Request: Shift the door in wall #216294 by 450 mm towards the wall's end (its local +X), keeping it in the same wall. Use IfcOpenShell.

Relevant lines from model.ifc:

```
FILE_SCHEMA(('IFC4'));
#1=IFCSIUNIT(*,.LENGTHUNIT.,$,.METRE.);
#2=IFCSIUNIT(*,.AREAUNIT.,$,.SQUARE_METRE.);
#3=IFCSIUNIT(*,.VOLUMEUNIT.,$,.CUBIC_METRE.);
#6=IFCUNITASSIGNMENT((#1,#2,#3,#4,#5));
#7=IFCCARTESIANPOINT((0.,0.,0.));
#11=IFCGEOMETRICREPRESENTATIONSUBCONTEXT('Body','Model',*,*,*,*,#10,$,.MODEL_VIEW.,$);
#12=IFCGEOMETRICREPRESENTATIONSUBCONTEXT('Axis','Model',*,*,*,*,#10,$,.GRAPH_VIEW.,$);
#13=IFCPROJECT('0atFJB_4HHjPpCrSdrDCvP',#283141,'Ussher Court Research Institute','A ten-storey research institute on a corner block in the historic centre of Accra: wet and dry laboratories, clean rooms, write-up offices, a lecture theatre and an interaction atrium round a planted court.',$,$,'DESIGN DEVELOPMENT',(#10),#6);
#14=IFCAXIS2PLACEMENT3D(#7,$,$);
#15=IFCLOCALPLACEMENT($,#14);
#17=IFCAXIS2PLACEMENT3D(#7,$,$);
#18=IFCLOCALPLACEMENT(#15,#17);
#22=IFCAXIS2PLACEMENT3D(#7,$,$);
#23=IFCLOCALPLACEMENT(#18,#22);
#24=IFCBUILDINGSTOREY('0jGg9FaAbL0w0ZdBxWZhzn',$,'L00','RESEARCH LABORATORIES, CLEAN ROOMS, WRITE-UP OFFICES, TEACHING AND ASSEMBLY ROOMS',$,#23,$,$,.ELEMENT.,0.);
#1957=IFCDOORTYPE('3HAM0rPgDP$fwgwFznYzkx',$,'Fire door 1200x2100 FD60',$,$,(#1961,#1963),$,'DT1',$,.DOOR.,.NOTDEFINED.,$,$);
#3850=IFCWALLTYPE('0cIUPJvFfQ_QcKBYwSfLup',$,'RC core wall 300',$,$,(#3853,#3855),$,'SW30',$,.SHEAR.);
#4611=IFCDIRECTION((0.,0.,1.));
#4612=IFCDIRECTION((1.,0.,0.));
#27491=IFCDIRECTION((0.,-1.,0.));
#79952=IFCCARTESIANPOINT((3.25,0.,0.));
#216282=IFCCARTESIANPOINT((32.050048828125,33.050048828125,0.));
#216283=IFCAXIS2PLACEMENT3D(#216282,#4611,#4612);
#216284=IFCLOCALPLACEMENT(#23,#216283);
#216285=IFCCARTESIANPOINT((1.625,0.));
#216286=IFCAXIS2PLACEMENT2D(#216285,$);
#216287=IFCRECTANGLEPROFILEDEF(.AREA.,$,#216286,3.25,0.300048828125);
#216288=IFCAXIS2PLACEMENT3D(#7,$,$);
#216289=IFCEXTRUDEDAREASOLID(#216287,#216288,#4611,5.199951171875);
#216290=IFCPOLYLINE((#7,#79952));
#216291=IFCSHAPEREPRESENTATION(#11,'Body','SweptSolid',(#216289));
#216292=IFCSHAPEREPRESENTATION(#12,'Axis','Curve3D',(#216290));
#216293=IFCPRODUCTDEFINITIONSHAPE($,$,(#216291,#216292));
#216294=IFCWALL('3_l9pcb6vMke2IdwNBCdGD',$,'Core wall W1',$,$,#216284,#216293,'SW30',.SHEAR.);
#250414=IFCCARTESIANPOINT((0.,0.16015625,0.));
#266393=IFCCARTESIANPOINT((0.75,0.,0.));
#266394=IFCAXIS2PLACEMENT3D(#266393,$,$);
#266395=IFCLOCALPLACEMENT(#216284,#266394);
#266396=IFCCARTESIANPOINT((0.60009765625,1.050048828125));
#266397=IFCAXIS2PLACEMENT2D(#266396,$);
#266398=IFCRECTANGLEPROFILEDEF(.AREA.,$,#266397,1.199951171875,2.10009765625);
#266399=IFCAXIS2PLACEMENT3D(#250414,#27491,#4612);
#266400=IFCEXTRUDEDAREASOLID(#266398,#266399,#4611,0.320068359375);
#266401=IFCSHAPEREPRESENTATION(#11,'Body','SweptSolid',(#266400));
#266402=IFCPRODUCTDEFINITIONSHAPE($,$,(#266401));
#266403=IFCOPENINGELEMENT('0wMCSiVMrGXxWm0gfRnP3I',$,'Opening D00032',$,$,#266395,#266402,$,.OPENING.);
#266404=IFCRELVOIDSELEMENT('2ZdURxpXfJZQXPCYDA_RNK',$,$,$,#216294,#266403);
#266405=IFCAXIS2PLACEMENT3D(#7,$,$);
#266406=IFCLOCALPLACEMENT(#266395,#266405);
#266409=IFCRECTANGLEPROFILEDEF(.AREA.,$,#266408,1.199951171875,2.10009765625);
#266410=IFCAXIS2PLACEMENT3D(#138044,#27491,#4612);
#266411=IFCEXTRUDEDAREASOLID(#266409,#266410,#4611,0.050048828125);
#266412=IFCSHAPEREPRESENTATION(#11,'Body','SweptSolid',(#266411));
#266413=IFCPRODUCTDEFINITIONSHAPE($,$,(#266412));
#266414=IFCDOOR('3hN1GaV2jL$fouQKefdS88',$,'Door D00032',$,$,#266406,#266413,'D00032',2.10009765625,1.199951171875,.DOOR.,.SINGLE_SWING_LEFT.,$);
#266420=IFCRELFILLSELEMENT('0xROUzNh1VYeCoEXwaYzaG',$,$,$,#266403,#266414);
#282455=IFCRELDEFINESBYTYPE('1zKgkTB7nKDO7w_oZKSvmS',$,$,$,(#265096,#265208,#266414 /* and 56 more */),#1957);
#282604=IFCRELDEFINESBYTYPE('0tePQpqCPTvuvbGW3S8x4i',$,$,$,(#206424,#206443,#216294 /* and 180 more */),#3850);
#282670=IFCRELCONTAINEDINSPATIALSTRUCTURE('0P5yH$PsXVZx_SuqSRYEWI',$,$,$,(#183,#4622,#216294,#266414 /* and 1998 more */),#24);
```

```python
import ifcopenshell
import ifcopenshell.api.geometry
import ifcopenshell.util.placement
import ifcopenshell.util.unit

model = ifcopenshell.open("model.ifc")
unit_scale = ifcopenshell.util.unit.calculate_unit_scale(model)

door = model.by_id(266414)
opening = door.FillsVoids[0].RelatingOpeningElement
wall = opening.VoidsElements[0].RelatingBuildingElement

wall_matrix = ifcopenshell.util.placement.get_local_placement(wall.ObjectPlacement)
shift = wall_matrix[:3, 0] * 0.45 / unit_scale
before = ifcopenshell.util.placement.get_local_placement(door.ObjectPlacement)[:3, 3].copy()

# The door is placed relative to its opening, so it follows when the opening moves.
matrix = ifcopenshell.util.placement.get_local_placement(opening.ObjectPlacement)
matrix[:3, 3] += shift
ifcopenshell.api.geometry.edit_object_placement(
    model, product=opening, matrix=matrix, is_si=False, should_transform_children=True
)

after = ifcopenshell.util.placement.get_local_placement(door.ObjectPlacement)[:3, 3]
print("door moved by", (after - before).round(3) + 0.0)

model.write("model_rev.ifc")
```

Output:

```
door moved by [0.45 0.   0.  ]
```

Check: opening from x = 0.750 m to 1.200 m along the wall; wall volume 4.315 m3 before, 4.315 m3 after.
